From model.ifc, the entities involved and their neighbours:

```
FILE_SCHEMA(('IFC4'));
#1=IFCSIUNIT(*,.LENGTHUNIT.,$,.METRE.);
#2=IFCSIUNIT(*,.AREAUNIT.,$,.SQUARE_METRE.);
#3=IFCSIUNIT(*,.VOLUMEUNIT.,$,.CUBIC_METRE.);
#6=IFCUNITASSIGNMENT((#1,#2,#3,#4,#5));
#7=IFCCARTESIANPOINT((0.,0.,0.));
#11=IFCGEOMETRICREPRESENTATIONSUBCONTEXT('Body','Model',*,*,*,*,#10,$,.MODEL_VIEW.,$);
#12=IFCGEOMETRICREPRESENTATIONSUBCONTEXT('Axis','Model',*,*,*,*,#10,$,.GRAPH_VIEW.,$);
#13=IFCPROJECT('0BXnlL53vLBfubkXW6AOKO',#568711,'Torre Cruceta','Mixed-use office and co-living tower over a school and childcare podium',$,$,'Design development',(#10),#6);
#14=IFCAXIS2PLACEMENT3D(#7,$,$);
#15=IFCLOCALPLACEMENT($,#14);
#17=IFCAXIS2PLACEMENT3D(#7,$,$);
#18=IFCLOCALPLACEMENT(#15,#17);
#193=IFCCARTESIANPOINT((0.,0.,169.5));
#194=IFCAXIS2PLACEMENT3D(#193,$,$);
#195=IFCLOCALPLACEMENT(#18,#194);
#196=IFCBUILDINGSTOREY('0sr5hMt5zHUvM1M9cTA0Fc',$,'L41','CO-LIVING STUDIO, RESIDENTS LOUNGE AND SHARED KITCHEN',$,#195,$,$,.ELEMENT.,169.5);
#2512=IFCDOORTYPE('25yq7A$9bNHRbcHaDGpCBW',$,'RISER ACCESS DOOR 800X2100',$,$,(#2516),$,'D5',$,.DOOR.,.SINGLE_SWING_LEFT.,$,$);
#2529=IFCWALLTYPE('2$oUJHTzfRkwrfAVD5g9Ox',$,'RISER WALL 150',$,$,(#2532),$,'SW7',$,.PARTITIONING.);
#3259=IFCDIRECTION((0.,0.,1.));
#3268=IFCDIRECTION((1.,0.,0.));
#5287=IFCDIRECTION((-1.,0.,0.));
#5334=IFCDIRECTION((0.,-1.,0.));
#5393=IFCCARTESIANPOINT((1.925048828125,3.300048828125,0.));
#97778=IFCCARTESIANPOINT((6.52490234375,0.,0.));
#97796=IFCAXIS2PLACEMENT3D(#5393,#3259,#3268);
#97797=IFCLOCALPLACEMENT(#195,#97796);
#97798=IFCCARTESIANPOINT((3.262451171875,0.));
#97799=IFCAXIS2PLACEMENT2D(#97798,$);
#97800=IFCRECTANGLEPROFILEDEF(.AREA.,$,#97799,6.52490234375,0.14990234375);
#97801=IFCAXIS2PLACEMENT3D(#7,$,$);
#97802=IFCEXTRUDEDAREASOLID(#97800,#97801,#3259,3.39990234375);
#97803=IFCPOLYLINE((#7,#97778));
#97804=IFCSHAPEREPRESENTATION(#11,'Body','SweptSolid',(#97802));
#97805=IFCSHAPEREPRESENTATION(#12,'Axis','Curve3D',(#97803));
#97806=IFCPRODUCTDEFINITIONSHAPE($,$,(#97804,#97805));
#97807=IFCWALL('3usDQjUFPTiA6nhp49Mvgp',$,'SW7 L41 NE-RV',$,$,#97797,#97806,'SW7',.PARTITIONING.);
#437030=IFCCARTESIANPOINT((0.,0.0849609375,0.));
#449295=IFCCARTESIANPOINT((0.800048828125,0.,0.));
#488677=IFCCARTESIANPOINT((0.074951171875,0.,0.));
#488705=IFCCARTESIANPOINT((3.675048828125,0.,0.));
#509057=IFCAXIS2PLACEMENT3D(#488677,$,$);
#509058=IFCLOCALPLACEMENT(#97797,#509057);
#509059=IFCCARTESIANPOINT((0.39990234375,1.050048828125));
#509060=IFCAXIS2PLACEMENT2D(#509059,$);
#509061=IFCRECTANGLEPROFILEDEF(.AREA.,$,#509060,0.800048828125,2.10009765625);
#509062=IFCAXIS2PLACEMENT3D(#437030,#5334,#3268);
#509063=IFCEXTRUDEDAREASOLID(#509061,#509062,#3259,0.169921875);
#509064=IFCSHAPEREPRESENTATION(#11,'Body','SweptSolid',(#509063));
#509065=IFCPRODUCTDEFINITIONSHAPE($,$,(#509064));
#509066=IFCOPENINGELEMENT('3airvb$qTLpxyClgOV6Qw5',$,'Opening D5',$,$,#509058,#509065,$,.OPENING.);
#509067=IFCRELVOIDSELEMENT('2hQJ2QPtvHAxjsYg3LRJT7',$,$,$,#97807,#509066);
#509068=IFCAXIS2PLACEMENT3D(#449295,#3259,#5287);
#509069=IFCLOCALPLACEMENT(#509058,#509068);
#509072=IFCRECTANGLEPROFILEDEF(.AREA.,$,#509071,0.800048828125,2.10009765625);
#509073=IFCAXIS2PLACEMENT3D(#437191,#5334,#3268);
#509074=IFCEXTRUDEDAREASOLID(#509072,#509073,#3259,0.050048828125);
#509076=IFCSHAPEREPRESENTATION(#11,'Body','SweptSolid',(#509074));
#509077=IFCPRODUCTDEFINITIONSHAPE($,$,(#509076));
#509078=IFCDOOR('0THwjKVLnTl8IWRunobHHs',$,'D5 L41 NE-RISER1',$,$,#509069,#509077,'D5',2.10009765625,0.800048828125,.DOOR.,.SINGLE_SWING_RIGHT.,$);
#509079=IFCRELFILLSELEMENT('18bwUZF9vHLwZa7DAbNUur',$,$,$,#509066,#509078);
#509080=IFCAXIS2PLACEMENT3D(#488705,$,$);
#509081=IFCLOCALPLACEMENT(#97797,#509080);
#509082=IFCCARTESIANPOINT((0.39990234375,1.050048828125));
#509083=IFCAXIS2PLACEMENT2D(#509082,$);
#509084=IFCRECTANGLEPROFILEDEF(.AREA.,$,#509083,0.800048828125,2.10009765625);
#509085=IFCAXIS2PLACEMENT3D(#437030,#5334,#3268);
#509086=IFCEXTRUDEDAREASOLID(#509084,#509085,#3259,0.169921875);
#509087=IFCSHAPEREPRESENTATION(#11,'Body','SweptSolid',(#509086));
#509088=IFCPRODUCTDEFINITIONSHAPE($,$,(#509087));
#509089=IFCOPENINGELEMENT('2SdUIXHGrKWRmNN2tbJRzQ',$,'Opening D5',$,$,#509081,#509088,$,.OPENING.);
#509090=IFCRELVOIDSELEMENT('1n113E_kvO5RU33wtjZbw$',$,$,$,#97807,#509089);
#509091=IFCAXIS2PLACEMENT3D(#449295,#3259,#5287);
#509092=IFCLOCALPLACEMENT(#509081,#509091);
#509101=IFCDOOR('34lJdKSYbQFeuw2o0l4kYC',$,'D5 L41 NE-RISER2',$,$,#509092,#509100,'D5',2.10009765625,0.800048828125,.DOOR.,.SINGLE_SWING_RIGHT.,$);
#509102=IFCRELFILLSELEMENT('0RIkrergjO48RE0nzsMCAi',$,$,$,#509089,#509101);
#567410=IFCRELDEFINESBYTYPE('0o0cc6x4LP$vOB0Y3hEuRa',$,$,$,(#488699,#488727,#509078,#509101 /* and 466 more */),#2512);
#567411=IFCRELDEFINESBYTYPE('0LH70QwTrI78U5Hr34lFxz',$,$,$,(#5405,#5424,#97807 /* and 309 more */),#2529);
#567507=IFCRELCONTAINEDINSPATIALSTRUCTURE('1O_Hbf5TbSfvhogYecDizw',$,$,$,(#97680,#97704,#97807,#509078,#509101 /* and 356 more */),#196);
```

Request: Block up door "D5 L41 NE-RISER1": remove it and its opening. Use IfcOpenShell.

```python
import ifcopenshell
import ifcopenshell.api.feature
import ifcopenshell.api.root
import ifcopenshell.geom
import ifcopenshell.util.shape

model = ifcopenshell.open("model.ifc")
settings = ifcopenshell.geom.settings()


def volume(element):
    """Net volume in cubic metres, openings subtracted."""
    shape = ifcopenshell.geom.create_shape(settings, element)
    return ifcopenshell.util.shape.get_volume(shape.geometry)


door = model.by_guid("0THwjKVLnTl8IWRunobHHs")
opening = door.FillsVoids[0].RelatingOpeningElement
wall = opening.VoidsElements[0].RelatingBuildingElement
before = volume(wall)

ifcopenshell.api.root.remove_product(model, product=door)
ifcopenshell.api.feature.remove_feature(model, feature=opening)

after = volume(wall)

print(f"wall volume {before:.3f} -> {after:.3f} m3")

model.write("model_edited.ifc")
```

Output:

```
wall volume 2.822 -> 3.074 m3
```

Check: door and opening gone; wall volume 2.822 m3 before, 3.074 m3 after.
